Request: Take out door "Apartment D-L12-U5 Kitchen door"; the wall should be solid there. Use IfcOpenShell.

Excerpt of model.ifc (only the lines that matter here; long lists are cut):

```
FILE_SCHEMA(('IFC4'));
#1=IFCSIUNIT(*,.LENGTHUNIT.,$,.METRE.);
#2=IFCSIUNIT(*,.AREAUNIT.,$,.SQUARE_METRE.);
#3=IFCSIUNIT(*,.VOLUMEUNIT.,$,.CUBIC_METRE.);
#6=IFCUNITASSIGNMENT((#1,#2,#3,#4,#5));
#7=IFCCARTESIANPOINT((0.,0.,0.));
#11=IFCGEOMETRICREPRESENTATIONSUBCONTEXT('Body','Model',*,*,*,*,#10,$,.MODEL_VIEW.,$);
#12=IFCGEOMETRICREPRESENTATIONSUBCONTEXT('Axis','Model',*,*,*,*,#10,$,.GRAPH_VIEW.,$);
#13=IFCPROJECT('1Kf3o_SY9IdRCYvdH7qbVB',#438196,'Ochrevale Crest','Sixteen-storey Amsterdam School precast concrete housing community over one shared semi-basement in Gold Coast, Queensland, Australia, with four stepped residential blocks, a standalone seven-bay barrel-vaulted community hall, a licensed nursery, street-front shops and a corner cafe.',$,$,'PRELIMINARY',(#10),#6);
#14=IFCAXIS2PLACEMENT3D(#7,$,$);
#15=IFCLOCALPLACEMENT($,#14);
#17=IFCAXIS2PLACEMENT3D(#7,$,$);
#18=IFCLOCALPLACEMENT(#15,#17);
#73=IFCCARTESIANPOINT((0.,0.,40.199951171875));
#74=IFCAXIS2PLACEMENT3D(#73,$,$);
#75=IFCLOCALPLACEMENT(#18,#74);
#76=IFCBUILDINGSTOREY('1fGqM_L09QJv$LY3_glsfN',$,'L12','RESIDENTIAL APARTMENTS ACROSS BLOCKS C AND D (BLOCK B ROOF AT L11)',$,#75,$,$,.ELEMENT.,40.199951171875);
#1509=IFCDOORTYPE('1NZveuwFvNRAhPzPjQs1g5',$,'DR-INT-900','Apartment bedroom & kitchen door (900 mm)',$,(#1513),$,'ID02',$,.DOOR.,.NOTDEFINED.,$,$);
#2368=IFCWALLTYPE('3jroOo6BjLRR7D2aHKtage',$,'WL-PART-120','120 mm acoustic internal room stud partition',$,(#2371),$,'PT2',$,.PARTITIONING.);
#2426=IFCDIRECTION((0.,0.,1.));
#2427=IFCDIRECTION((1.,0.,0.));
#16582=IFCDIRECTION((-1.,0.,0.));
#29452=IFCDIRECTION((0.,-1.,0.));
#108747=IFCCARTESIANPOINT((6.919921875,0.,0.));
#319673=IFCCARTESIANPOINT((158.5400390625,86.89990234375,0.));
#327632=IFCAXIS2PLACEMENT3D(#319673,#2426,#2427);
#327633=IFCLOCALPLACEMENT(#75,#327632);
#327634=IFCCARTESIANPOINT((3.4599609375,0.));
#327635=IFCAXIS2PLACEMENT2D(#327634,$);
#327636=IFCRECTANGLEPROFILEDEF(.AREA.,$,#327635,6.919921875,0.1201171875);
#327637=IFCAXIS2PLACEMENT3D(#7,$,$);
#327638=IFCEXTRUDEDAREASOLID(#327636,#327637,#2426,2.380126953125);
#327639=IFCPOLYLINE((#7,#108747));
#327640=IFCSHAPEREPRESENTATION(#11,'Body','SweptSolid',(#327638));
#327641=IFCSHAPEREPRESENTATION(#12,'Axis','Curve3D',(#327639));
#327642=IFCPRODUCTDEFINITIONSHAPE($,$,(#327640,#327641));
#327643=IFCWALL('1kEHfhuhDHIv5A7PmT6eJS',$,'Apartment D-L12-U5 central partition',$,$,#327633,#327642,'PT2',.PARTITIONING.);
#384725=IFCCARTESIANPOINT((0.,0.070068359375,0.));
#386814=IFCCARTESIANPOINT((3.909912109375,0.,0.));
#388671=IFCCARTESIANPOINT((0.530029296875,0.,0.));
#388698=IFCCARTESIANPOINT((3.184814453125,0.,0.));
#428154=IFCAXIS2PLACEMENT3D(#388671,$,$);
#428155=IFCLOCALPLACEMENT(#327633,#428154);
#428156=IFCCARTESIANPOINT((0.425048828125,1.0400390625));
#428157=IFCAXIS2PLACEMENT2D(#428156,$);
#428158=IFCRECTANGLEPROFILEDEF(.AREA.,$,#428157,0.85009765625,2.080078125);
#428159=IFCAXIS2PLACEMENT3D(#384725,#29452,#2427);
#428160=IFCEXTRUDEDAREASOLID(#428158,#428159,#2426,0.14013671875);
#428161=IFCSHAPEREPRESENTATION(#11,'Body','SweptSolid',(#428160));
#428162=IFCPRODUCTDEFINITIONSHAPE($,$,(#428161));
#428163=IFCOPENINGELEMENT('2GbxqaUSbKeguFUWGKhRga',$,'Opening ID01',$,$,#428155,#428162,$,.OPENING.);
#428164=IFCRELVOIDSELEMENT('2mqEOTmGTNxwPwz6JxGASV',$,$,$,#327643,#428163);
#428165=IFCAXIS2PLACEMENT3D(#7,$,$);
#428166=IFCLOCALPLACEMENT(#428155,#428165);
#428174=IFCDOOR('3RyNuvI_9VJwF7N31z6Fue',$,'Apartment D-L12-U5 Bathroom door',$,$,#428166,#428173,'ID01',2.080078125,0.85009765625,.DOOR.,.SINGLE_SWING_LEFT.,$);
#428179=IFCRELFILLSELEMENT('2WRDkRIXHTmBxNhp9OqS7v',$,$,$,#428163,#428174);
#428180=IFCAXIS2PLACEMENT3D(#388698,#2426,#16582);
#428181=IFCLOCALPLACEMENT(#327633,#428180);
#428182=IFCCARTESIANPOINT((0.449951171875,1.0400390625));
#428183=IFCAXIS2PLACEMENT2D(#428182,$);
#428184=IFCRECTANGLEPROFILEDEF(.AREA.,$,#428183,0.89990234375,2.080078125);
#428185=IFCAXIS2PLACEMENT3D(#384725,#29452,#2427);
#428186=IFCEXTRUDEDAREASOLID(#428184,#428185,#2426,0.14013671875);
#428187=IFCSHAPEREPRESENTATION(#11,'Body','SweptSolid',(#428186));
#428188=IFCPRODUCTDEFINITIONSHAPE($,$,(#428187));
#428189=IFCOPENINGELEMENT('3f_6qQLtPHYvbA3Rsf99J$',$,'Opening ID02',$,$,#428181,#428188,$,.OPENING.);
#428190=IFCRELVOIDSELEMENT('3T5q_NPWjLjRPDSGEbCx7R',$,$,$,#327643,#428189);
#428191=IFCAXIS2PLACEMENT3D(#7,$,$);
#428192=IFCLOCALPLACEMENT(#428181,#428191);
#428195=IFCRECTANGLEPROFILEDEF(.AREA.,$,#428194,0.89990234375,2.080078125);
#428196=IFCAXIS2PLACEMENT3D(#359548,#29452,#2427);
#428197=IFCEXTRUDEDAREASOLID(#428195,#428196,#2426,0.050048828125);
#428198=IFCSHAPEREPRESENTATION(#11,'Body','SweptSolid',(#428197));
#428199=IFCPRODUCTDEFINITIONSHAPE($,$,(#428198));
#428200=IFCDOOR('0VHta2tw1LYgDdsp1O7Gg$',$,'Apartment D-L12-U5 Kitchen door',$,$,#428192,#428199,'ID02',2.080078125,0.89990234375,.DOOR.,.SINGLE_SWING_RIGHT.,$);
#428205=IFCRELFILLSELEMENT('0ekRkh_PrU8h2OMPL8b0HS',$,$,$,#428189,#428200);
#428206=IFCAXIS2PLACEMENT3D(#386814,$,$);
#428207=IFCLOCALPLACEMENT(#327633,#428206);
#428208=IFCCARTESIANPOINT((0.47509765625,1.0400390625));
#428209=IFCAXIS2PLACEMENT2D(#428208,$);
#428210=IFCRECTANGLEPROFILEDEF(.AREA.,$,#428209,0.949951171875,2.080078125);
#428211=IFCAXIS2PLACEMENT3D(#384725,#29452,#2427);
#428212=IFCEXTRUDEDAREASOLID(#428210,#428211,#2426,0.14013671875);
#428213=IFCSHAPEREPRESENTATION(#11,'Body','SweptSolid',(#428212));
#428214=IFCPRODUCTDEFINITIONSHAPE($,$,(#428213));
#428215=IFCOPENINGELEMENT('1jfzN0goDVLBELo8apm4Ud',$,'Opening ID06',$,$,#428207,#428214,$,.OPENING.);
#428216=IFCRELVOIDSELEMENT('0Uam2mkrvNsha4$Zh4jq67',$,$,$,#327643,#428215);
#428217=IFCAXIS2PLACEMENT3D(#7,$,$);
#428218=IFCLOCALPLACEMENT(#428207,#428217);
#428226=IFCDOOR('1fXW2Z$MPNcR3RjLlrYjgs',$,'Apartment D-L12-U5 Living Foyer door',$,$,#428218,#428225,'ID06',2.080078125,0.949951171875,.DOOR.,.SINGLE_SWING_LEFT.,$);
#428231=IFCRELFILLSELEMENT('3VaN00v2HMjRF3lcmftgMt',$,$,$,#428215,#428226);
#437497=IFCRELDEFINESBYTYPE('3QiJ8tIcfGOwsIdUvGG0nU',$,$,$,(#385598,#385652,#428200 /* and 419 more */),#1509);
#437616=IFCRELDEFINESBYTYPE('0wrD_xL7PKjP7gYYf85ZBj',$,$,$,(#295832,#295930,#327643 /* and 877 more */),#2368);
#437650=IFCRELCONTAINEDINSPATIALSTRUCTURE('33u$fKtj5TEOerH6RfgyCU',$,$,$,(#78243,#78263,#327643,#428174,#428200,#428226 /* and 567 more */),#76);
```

```python
import ifcopenshell
import ifcopenshell.api.feature
import ifcopenshell.api.root
import ifcopenshell.geom
import ifcopenshell.util.shape

model = ifcopenshell.open("model.ifc")
settings = ifcopenshell.geom.settings()


def volume(element):
    """Net volume in cubic metres, openings subtracted."""
    shape = ifcopenshell.geom.create_shape(settings, element)
    return ifcopenshell.util.shape.get_volume(shape.geometry)


door = model.by_id(428200)
opening = door.FillsVoids[0].RelatingOpeningElement
wall = opening.VoidsElements[0].RelatingBuildingElement
before = volume(wall)

ifcopenshell.api.root.remove_product(model, product=door)
ifcopenshell.api.feature.remove_feature(model, feature=opening)

after = volume(wall)

print(f"wall volume {before:.3f} -> {after:.3f} m3")

model.write("model_updated.ifc")
```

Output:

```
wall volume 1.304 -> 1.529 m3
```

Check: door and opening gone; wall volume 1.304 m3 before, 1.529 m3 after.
